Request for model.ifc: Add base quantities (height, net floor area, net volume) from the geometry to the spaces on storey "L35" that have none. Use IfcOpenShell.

First a look at what the model holds.

```python
import ifcopenshell
import ifcopenshell.util.element
import ifcopenshell.util.unit

model = ifcopenshell.open("model.ifc")
print(model.schema)
for unit_type in ("LENGTHUNIT", "AREAUNIT", "VOLUMEUNIT"):
    print(unit_type, ifcopenshell.util.unit.calculate_unit_scale(model, unit_type))
storey = next(s for s in model.by_type("IfcBuildingStorey") if s.Name == "L35")
spaces = [e for e in ifcopenshell.util.element.get_decomposition(storey) if e.is_a("IfcSpace")]
for e in sorted(spaces, key=lambda e: e.id()):
    print(e.id(), e.is_a(), e.Name, list(ifcopenshell.util.element.get_psets(e, qtos_only=True)), sep=" | ")
```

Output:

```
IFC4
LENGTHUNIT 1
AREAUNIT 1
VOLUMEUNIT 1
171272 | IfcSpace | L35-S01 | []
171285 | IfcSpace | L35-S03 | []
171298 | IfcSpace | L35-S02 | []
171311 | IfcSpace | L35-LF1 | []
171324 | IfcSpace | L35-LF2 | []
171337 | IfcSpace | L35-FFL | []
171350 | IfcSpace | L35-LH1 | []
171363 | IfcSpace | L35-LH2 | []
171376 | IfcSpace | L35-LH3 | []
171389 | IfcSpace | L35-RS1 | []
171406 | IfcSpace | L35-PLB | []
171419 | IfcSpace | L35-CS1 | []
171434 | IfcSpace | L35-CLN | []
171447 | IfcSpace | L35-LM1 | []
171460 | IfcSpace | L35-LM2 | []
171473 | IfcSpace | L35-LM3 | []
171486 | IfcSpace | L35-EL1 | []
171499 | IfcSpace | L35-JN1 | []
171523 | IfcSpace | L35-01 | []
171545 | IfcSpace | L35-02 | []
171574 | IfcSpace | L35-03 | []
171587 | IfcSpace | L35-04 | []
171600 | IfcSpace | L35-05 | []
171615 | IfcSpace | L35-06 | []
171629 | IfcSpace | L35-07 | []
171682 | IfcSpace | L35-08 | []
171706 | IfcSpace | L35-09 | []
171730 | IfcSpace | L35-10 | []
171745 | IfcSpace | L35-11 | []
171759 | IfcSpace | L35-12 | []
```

```python
import ifcopenshell
import ifcopenshell.api.pset
import ifcopenshell.geom
import ifcopenshell.util.element
import ifcopenshell.util.shape
import ifcopenshell.util.unit

model = ifcopenshell.open("model.ifc")
unit_scale = ifcopenshell.util.unit.calculate_unit_scale(model)
area_scale = ifcopenshell.util.unit.calculate_unit_scale(model, "AREAUNIT")
volume_scale = ifcopenshell.util.unit.calculate_unit_scale(model, "VOLUMEUNIT")
settings = ifcopenshell.geom.settings()

storey = next(s for s in model.by_type("IfcBuildingStorey") if s.Name == "L35")
spaces = [e for e in ifcopenshell.util.element.get_decomposition(storey) if e.is_a("IfcSpace")]

for e in sorted(spaces, key=lambda e: e.id()):
    if ifcopenshell.util.element.get_psets(e, qtos_only=True, should_inherit=False):
        continue
    # Geometry comes back in metres, in the element's own axes.
    shape = ifcopenshell.geom.create_shape(settings, e)
    values = {
        "Height": ifcopenshell.util.shape.get_z(shape.geometry) / unit_scale,
        "NetFloorArea": ifcopenshell.util.shape.get_footprint_area(shape.geometry) / area_scale,
        "NetVolume": ifcopenshell.util.shape.get_volume(shape.geometry) / volume_scale,
    }
    qto = ifcopenshell.api.pset.add_qto(model, product=e, name="Qto_SpaceBaseQuantities")
    ifcopenshell.api.pset.edit_qto(model, qto=qto, properties=values)
    print(e.id(), {k: round(v, 3) for k, v in values.items()})

model.write("model_updated.ifc")
```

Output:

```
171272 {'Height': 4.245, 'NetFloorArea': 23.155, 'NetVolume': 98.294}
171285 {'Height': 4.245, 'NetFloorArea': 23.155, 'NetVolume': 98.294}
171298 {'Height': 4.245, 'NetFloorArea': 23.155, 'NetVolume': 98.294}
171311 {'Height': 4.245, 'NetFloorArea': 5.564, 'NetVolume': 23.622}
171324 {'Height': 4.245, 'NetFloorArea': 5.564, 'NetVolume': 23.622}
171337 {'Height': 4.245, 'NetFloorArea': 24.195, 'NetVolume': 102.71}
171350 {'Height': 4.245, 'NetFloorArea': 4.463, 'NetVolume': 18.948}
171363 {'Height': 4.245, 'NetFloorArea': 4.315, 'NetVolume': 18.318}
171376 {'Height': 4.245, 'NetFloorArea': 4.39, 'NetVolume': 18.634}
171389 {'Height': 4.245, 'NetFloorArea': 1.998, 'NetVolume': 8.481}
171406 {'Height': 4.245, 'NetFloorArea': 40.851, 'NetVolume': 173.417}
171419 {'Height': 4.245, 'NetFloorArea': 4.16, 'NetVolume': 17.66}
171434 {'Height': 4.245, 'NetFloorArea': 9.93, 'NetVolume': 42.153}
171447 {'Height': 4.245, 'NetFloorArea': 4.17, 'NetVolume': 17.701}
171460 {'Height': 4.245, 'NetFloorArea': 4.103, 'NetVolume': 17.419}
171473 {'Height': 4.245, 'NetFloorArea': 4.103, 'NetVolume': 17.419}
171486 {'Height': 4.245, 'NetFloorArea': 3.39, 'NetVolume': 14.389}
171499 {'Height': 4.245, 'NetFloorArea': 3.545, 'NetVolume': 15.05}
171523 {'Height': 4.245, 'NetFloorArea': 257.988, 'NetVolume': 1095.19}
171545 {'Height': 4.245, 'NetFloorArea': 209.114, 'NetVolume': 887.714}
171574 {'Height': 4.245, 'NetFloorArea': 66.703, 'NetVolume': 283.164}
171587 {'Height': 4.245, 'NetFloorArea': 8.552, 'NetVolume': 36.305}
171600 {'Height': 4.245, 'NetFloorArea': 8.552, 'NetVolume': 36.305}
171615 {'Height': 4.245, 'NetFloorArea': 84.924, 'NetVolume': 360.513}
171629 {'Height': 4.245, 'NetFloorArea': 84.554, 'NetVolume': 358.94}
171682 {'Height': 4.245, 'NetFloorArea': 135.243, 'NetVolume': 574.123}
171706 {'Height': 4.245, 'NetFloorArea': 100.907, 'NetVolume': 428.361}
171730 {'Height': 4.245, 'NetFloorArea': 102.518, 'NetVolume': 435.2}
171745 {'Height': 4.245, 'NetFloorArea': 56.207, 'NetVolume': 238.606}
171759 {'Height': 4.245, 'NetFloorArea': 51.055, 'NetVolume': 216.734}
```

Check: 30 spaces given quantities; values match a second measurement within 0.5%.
